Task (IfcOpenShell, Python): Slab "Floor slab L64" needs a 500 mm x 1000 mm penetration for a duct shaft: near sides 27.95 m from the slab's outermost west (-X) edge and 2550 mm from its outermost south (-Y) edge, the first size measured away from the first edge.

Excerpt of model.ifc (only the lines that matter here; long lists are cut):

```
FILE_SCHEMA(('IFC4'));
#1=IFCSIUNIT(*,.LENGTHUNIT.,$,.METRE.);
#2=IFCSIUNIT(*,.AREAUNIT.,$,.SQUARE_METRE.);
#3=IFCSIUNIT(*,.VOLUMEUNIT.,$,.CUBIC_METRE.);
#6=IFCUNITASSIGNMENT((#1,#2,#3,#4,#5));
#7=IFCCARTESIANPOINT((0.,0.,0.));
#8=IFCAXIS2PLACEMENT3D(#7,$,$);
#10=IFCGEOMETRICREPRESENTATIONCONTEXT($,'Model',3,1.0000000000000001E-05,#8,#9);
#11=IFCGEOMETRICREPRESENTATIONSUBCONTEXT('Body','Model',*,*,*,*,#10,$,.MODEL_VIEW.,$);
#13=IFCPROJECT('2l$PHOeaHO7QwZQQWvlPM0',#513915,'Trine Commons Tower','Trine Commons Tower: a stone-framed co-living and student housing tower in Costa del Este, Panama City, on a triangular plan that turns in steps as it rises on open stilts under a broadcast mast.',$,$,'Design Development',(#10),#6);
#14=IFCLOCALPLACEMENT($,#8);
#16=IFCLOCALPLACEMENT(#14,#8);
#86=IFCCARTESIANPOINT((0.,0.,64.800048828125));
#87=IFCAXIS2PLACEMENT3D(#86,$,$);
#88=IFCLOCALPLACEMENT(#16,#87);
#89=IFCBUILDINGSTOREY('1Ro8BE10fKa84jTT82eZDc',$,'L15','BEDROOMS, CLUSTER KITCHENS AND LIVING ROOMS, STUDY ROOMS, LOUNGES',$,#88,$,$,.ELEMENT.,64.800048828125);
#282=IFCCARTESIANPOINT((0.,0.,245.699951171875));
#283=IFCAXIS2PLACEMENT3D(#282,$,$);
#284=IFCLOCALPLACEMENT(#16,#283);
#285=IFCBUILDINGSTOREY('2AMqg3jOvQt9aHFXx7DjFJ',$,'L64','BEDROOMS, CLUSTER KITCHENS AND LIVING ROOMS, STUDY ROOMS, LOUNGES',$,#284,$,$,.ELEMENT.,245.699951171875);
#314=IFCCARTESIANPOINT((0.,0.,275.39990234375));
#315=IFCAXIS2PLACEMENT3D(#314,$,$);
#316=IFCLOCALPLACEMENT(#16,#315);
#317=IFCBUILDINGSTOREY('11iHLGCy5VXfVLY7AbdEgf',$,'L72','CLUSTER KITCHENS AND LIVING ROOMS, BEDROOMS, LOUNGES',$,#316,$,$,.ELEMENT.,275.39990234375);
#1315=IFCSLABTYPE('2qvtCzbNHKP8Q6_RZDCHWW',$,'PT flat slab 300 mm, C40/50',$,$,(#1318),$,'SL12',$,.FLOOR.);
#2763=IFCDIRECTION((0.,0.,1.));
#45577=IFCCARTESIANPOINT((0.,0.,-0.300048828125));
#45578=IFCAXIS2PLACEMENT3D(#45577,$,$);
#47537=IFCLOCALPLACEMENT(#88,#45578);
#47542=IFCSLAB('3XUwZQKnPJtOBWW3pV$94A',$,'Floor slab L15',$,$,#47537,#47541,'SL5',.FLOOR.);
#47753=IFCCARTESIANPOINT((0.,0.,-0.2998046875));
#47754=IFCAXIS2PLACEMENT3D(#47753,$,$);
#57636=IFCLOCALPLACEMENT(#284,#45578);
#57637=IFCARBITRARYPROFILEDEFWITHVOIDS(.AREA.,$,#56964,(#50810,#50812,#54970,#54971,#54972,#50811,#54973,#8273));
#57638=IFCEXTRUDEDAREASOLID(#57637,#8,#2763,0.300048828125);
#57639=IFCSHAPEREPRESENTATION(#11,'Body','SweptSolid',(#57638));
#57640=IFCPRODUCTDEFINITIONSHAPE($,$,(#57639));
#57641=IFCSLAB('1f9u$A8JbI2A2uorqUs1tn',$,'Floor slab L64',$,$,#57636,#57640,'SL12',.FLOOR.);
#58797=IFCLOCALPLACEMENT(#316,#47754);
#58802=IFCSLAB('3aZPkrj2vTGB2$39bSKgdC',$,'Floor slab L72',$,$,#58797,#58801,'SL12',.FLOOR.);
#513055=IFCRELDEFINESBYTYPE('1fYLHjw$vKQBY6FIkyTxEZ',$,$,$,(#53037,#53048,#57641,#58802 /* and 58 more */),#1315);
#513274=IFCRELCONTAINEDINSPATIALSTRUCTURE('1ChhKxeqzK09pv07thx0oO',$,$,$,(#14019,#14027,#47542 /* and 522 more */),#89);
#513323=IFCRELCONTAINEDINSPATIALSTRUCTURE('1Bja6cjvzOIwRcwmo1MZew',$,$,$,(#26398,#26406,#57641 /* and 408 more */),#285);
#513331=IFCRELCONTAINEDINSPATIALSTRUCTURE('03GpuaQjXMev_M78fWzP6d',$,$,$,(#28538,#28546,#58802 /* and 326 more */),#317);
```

```python
import numpy as np
import ifcopenshell
import ifcopenshell.api.feature
import ifcopenshell.api.geometry
import ifcopenshell.api.root
import ifcopenshell.geom
import ifcopenshell.util.placement
import ifcopenshell.util.representation
import ifcopenshell.util.shape
import ifcopenshell.util.unit

model = ifcopenshell.open("model.ifc")
unit_scale = ifcopenshell.util.unit.calculate_unit_scale(model)
settings = ifcopenshell.geom.settings()


def volume(element):
    """Net volume in cubic metres, openings subtracted."""
    shape = ifcopenshell.geom.create_shape(settings, element)
    return ifcopenshell.util.shape.get_volume(shape.geometry)


slab = model.by_guid("1f9u$A8JbI2A2uorqUs1tn")
before = volume(slab)

# Extent in the slab's own axes, in metres. The edges named are its -X and -Y sides.
slab_shape = ifcopenshell.geom.create_shape(settings, slab)
vertices = ifcopenshell.util.shape.get_vertices(slab_shape.geometry)
x_min, y_min, bottom = vertices.min(axis=0)
top = vertices[:, 2].max()

opening = ifcopenshell.api.root.create_entity(model, ifc_class="IfcOpeningElement", name="Duct shaft opening", predefined_type="OPENING")
context = ifcopenshell.util.representation.get_context(model, "Model", "Body", "MODEL_VIEW")
width, depth = 0.5, 1
outline = [(0.0, 0.0), (width, 0.0), (width, depth), (0.0, depth), (0.0, 0.0)]
# Overshoot both faces by 50 mm so the cut is clean.
shape = ifcopenshell.api.geometry.add_slab_representation(
    model, context=context, depth=top - bottom + 0.1, polyline=outline
)
ifcopenshell.api.geometry.assign_representation(model, product=opening, representation=shape)

matrix = ifcopenshell.util.placement.get_local_placement(slab.ObjectPlacement)
matrix[:, 3] = matrix @ np.append(np.array([x_min + 27.95, y_min + 2.55, bottom - 0.05]) / unit_scale, 1.0)
ifcopenshell.api.geometry.edit_object_placement(model, product=opening, matrix=matrix, is_si=False)
ifcopenshell.api.feature.add_feature(model, feature=opening, element=slab)

after = volume(slab)

print(f"slab volume {before:.3f} -> {after:.3f} m3")

model.write("model_v2.ifc")
```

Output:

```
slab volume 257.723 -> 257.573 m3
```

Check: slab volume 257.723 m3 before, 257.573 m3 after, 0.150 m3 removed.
